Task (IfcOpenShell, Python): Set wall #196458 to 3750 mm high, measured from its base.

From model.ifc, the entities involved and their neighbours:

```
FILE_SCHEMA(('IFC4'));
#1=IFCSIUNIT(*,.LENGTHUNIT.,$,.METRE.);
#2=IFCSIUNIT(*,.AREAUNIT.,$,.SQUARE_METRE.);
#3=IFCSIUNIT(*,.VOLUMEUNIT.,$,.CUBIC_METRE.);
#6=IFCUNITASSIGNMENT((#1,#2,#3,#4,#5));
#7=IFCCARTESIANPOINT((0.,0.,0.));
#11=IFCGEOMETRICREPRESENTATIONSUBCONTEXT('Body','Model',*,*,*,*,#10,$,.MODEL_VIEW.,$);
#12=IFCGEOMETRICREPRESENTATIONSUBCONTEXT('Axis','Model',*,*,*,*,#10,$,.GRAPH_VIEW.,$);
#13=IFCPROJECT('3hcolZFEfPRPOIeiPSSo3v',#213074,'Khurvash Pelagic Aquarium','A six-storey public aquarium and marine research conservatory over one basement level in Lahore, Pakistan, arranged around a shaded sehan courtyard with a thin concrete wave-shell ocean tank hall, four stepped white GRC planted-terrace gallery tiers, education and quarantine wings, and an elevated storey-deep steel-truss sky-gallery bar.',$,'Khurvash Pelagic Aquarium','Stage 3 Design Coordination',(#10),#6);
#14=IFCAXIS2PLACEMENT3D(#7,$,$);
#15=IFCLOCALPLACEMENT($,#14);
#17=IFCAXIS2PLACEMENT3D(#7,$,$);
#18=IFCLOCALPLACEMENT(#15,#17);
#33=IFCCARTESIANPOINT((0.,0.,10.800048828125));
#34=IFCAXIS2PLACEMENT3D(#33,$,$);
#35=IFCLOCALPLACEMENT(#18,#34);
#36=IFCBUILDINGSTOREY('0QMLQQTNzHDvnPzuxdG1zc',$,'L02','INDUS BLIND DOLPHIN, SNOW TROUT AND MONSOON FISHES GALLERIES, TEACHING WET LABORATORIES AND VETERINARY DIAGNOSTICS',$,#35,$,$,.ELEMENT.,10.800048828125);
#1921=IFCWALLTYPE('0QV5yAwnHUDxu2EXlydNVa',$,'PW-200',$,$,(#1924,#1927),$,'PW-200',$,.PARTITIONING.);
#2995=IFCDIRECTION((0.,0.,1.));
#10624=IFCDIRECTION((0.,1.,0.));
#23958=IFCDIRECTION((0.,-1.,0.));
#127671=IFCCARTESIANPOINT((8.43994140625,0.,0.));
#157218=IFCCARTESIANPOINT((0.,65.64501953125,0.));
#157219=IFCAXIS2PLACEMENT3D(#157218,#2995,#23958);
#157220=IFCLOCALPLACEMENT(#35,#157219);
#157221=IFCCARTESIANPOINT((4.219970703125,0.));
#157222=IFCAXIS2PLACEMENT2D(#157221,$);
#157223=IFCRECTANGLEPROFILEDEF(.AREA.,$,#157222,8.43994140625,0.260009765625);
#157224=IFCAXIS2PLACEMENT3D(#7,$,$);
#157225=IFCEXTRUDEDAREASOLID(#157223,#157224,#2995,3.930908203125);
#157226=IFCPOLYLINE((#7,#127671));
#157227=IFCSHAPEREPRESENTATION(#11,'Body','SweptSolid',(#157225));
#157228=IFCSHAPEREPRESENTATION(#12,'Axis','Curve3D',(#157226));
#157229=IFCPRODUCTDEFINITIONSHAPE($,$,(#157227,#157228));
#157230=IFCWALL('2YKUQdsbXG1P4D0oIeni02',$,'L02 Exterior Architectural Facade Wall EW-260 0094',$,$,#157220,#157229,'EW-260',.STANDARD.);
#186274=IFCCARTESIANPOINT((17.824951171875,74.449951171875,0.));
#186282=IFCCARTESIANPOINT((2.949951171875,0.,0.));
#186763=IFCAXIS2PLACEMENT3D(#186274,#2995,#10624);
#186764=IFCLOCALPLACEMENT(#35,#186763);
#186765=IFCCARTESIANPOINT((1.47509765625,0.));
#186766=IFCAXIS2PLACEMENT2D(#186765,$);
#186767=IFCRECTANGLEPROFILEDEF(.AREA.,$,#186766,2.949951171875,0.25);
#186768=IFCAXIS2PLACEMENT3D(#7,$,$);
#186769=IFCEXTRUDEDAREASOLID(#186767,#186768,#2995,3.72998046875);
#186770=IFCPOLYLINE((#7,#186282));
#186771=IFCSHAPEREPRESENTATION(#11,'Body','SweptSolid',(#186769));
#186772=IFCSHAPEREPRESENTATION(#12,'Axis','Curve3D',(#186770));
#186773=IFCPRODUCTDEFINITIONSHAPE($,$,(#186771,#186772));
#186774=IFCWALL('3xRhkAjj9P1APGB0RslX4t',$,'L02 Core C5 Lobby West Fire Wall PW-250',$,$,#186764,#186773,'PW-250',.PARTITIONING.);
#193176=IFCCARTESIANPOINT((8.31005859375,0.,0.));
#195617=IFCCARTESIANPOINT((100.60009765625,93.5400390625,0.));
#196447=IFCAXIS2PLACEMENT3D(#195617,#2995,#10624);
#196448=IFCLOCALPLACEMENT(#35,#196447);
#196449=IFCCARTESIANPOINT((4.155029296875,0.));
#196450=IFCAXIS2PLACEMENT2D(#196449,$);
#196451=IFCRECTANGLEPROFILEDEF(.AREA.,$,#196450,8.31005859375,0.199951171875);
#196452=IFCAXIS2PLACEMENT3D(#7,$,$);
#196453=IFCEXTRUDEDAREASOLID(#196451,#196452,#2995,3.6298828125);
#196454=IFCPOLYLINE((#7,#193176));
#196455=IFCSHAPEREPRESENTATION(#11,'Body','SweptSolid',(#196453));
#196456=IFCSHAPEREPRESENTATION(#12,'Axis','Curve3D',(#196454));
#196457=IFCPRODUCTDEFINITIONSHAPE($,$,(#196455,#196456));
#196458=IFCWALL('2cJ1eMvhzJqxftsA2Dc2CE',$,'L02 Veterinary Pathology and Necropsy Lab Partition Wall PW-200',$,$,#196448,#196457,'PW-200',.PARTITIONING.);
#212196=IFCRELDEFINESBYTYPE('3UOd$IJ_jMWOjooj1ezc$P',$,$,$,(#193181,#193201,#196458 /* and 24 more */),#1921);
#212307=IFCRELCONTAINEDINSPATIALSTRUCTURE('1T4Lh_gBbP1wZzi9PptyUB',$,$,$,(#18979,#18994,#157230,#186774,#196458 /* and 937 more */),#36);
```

```python
import ifcopenshell
import ifcopenshell.geom
import ifcopenshell.util.representation
import ifcopenshell.util.shape

model = ifcopenshell.open("model.ifc")
settings = ifcopenshell.geom.settings()


def volume(element):
    """Net volume in cubic metres, openings subtracted."""
    shape = ifcopenshell.geom.create_shape(settings, element)
    return ifcopenshell.util.shape.get_volume(shape.geometry)


wall = model.by_guid("2cJ1eMvhzJqxftsA2Dc2CE")
before = volume(wall)

body = ifcopenshell.util.representation.get_representation(wall, "Model", "Body")
solid = body.Items[0]
old_height = solid.Depth
solid.Depth = 3.75
after = volume(wall)

print(f"height {old_height:g} -> {solid.Depth:g}, volume {before:.3f} -> {after:.3f} m3")

model.write("model_edited.ifc")
```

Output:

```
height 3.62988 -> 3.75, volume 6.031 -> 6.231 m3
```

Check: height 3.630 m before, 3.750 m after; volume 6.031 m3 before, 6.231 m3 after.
